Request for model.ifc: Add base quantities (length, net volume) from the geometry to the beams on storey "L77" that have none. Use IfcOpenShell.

First a look at what the model holds.

```python
import ifcopenshell
import ifcopenshell.util.element
import ifcopenshell.util.unit

model = ifcopenshell.open("model.ifc")
print(model.schema)
for unit_type in ("LENGTHUNIT", "AREAUNIT", "VOLUMEUNIT"):
    print(unit_type, ifcopenshell.util.unit.calculate_unit_scale(model, unit_type))
storey = next(s for s in model.by_type("IfcBuildingStorey") if s.Name == "L77")
beams = [e for e in ifcopenshell.util.element.get_decomposition(storey) if e.is_a("IfcBeam")]
for e in sorted(beams, key=lambda e: e.id()):
    print(e.id(), e.is_a(), e.Name, list(ifcopenshell.util.element.get_psets(e, qtos_only=True)), sep=" | ")
```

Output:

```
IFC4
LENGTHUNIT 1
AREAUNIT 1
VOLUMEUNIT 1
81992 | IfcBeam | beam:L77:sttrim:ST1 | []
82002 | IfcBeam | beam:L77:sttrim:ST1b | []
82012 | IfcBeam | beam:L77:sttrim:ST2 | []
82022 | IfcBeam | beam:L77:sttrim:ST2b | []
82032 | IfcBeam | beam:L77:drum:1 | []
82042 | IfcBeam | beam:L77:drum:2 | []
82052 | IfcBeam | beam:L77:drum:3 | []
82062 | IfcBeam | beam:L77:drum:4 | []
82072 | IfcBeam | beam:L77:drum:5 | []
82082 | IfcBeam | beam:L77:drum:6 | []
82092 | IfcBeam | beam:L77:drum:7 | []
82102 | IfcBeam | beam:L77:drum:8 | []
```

```python
import ifcopenshell
import ifcopenshell.api.pset
import ifcopenshell.geom
import ifcopenshell.util.element
import ifcopenshell.util.shape
import ifcopenshell.util.unit

model = ifcopenshell.open("model.ifc")
unit_scale = ifcopenshell.util.unit.calculate_unit_scale(model)
volume_scale = ifcopenshell.util.unit.calculate_unit_scale(model, "VOLUMEUNIT")
settings = ifcopenshell.geom.settings()

storey = next(s for s in model.by_type("IfcBuildingStorey") if s.Name == "L77")
beams = [e for e in ifcopenshell.util.element.get_decomposition(storey) if e.is_a("IfcBeam")]

for e in sorted(beams, key=lambda e: e.id()):
    if ifcopenshell.util.element.get_psets(e, qtos_only=True, should_inherit=False):
        continue
    # Geometry comes back in metres, in the element's own axes.
    shape = ifcopenshell.geom.create_shape(settings, e)
    values = {
        "Length": ifcopenshell.util.shape.get_max_xyz(shape.geometry) / unit_scale,
        "NetVolume": ifcopenshell.util.shape.get_volume(shape.geometry) / volume_scale,
    }
    qto = ifcopenshell.api.pset.add_qto(model, product=e, name="Qto_BeamBaseQuantities")
    ifcopenshell.api.pset.edit_qto(model, qto=qto, properties=values)
    print(e.id(), {k: round(v, 3) for k, v in values.items()})

model.write("model-out.ifc")
```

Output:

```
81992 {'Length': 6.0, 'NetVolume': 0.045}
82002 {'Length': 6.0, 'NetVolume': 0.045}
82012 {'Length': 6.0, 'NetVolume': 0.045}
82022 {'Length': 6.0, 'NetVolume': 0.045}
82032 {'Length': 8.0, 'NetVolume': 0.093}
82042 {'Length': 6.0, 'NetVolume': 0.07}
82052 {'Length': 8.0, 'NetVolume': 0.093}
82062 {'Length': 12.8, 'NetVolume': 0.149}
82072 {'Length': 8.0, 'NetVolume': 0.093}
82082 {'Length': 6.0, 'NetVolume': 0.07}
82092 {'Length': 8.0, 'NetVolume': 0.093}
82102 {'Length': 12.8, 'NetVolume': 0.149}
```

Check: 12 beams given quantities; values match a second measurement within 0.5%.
